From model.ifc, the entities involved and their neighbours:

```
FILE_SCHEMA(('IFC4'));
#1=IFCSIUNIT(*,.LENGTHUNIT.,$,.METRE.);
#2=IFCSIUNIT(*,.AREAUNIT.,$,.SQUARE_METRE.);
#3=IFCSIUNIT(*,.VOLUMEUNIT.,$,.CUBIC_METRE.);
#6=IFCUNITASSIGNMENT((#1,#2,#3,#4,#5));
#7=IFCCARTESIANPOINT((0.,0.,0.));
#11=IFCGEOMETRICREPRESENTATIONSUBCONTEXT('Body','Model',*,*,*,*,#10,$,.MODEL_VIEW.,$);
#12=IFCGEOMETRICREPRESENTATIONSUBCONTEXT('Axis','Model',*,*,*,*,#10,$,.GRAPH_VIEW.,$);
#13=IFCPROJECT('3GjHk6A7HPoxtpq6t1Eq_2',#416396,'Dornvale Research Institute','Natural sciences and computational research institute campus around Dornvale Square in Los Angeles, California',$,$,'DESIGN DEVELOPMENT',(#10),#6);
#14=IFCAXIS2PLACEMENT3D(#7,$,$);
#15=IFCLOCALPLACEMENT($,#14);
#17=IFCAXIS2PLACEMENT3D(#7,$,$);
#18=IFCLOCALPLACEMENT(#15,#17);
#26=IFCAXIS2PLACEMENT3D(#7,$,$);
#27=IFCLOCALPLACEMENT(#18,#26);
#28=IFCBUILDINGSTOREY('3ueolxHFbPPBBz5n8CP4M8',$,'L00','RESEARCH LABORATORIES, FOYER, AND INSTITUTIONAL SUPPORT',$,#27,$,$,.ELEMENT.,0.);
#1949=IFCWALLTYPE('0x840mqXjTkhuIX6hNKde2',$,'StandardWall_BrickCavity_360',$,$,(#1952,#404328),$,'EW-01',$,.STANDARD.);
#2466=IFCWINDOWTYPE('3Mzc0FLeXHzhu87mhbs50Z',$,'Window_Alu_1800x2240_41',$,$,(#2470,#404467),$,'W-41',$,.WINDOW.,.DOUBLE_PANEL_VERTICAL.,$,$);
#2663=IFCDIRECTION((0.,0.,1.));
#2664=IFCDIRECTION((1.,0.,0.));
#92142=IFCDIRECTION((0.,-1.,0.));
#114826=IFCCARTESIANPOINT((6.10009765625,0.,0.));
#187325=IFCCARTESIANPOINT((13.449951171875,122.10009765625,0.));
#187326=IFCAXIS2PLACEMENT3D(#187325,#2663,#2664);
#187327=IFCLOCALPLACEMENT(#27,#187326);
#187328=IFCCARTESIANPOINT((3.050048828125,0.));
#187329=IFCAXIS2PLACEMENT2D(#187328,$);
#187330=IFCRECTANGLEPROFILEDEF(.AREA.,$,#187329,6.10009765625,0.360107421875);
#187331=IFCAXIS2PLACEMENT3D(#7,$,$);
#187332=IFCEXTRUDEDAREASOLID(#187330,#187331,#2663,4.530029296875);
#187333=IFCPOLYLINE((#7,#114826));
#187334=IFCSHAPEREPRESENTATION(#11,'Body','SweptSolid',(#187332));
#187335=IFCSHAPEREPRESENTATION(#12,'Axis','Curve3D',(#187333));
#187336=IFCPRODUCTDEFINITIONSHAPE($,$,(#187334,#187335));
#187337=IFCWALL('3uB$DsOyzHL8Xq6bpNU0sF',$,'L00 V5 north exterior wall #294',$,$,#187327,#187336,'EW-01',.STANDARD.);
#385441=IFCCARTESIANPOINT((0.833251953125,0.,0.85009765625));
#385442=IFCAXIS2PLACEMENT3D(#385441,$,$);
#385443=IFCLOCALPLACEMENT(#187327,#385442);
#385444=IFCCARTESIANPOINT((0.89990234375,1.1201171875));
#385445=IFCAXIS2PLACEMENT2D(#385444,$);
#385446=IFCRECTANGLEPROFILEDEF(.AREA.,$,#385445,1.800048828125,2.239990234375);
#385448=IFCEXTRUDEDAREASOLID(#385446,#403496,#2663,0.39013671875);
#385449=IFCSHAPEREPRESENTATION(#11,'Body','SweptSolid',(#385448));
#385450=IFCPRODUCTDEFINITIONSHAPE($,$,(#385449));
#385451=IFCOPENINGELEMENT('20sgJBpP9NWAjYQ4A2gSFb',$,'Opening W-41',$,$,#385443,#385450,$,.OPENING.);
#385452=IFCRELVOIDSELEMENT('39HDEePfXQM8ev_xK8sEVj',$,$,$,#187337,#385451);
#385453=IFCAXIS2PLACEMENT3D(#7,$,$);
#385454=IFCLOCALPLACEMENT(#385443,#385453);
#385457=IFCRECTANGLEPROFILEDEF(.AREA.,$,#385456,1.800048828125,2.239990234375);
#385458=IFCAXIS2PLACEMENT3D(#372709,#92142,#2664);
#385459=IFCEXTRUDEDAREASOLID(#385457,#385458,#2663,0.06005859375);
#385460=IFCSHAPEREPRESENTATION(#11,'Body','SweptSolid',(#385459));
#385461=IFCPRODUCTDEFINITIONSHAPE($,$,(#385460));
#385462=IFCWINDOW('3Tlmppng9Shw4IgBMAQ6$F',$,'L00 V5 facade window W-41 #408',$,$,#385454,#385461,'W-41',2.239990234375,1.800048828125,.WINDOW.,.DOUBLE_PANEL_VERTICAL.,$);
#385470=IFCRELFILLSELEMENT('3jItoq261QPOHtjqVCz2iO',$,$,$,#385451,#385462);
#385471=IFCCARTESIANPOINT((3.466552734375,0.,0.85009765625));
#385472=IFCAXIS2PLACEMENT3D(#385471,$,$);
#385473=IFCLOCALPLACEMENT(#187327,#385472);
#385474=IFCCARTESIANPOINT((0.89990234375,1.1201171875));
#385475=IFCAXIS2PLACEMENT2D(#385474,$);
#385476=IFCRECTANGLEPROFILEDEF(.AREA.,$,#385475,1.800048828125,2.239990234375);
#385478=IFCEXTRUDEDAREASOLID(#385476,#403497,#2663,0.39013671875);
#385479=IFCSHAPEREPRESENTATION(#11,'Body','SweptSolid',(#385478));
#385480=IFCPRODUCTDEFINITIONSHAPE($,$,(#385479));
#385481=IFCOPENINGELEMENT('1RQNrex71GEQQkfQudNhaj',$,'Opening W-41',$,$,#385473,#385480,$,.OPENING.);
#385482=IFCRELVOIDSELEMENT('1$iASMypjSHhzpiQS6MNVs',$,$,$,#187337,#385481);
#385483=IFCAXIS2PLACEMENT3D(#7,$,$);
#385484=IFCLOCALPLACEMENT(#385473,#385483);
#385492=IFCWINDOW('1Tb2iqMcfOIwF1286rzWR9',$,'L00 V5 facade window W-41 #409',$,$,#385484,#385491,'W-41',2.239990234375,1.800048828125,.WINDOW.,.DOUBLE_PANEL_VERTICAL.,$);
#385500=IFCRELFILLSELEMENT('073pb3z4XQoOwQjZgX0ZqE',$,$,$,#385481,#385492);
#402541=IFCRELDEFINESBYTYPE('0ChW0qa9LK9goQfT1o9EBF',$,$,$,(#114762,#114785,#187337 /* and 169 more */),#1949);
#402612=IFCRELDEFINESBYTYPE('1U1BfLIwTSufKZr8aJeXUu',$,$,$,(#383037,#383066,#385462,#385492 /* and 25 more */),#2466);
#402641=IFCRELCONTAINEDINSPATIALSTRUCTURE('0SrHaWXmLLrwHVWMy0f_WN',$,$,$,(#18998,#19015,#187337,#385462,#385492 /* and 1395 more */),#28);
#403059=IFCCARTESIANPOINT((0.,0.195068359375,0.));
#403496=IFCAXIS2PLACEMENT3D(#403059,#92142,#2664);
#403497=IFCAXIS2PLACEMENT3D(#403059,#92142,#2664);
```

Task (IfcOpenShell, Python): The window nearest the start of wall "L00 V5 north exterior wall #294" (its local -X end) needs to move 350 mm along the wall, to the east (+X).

```python
import ifcopenshell
import ifcopenshell.api.geometry
import ifcopenshell.util.placement
import ifcopenshell.util.unit

model = ifcopenshell.open("model.ifc")
unit_scale = ifcopenshell.util.unit.calculate_unit_scale(model)

window = model.by_guid("3Tlmppng9Shw4IgBMAQ6$F")
opening = window.FillsVoids[0].RelatingOpeningElement
wall = opening.VoidsElements[0].RelatingBuildingElement

wall_matrix = ifcopenshell.util.placement.get_local_placement(wall.ObjectPlacement)
shift = wall_matrix[:3, 0] * 0.35 / unit_scale
before = ifcopenshell.util.placement.get_local_placement(window.ObjectPlacement)[:3, 3].copy()

# The window is placed relative to its opening, so it follows when the opening moves.
matrix = ifcopenshell.util.placement.get_local_placement(opening.ObjectPlacement)
matrix[:3, 3] += shift
ifcopenshell.api.geometry.edit_object_placement(
    model, product=opening, matrix=matrix, is_si=False, should_transform_children=True
)

after = ifcopenshell.util.placement.get_local_placement(window.ObjectPlacement)[:3, 3]
print("window moved by", (after - before).round(3) + 0.0)

model.write("model_v2.ifc")
```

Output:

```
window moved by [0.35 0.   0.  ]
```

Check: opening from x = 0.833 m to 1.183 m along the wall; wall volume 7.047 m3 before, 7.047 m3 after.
